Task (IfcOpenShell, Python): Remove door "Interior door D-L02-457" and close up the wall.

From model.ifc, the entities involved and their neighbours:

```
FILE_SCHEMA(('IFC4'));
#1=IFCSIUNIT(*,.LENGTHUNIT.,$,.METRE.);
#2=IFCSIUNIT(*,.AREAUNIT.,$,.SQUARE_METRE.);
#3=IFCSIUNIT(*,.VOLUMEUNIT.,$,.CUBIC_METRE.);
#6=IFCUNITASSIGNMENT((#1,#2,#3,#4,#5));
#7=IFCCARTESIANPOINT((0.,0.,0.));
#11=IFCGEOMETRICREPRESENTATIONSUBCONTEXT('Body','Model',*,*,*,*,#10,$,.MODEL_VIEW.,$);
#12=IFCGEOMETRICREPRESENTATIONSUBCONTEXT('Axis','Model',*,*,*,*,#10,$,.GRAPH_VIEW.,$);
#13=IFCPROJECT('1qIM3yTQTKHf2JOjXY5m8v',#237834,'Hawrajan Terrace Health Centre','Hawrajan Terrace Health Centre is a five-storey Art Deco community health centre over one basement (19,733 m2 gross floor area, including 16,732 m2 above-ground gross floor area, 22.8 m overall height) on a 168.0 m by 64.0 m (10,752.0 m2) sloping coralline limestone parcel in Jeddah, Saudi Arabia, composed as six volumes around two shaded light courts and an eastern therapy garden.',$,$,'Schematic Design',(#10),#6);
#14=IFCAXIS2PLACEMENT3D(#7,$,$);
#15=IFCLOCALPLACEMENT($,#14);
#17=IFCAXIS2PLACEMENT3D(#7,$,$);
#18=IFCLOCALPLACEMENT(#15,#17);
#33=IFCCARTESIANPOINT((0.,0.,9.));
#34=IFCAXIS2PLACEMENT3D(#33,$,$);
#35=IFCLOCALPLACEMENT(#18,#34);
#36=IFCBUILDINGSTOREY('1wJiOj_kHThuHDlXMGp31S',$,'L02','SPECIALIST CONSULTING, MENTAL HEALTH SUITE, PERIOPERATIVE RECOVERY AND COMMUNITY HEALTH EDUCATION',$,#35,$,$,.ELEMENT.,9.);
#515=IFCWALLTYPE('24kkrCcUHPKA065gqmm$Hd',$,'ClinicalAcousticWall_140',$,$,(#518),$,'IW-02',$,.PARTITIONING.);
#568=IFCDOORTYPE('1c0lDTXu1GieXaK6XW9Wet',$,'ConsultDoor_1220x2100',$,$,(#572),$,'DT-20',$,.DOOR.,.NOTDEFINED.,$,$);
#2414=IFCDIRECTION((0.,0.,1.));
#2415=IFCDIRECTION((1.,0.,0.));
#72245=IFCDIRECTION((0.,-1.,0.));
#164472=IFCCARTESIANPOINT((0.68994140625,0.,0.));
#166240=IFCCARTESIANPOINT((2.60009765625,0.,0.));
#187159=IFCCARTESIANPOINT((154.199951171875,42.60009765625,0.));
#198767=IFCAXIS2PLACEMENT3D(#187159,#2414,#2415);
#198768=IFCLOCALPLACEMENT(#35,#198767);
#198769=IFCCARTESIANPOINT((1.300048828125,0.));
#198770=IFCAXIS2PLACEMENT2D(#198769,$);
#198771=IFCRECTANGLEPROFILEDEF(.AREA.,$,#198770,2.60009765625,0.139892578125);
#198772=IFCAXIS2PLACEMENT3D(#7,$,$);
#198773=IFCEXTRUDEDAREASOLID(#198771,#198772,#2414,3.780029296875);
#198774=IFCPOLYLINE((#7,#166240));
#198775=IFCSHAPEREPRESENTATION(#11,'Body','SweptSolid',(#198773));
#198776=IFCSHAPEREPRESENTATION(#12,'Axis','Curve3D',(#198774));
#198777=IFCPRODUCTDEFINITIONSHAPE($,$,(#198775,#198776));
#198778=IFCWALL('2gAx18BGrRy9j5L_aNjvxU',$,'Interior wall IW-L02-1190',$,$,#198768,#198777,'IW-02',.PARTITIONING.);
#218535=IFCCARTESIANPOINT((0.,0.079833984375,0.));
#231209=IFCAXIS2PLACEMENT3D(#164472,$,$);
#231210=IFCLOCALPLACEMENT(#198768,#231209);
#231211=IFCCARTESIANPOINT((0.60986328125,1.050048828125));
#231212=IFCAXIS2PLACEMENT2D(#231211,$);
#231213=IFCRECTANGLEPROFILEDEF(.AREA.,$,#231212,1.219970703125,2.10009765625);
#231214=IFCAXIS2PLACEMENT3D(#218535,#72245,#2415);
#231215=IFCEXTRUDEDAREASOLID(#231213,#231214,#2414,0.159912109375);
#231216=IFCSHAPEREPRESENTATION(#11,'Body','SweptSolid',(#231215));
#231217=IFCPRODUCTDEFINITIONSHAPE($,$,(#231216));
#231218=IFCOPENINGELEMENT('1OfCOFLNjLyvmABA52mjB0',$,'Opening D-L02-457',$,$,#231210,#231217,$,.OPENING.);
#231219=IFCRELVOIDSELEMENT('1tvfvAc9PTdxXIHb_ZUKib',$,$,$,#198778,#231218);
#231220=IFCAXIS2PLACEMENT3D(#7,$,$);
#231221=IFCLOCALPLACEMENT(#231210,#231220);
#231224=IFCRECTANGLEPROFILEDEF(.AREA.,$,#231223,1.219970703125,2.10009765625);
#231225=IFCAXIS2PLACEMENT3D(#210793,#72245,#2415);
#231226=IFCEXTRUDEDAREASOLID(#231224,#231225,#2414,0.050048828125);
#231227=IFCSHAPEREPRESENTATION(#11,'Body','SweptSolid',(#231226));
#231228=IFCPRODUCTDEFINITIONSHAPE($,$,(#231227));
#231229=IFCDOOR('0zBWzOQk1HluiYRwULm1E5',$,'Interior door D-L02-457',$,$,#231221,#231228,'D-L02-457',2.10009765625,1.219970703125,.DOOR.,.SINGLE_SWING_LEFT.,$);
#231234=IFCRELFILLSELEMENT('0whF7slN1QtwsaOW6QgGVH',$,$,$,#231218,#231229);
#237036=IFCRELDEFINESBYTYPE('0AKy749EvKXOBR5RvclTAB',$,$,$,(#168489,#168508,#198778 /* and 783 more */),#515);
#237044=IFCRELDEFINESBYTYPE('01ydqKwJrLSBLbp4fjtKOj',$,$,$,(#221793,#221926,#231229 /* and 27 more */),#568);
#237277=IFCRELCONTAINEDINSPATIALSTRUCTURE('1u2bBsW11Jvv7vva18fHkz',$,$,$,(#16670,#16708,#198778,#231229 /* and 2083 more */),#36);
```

```python
import ifcopenshell
import ifcopenshell.api.feature
import ifcopenshell.api.root
import ifcopenshell.geom
import ifcopenshell.util.shape

model = ifcopenshell.open("model.ifc")
settings = ifcopenshell.geom.settings()


def volume(element):
    """Net volume in cubic metres, openings subtracted."""
    shape = ifcopenshell.geom.create_shape(settings, element)
    return ifcopenshell.util.shape.get_volume(shape.geometry)


door = model.by_guid("0zBWzOQk1HluiYRwULm1E5")
opening = door.FillsVoids[0].RelatingOpeningElement
wall = opening.VoidsElements[0].RelatingBuildingElement
before = volume(wall)

ifcopenshell.api.root.remove_product(model, product=door)
ifcopenshell.api.feature.remove_feature(model, feature=opening)

after = volume(wall)

print(f"wall volume {before:.3f} -> {after:.3f} m3")

model.write("model_updated.ifc")
```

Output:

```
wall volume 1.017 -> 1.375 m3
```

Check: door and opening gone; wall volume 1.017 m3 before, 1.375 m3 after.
